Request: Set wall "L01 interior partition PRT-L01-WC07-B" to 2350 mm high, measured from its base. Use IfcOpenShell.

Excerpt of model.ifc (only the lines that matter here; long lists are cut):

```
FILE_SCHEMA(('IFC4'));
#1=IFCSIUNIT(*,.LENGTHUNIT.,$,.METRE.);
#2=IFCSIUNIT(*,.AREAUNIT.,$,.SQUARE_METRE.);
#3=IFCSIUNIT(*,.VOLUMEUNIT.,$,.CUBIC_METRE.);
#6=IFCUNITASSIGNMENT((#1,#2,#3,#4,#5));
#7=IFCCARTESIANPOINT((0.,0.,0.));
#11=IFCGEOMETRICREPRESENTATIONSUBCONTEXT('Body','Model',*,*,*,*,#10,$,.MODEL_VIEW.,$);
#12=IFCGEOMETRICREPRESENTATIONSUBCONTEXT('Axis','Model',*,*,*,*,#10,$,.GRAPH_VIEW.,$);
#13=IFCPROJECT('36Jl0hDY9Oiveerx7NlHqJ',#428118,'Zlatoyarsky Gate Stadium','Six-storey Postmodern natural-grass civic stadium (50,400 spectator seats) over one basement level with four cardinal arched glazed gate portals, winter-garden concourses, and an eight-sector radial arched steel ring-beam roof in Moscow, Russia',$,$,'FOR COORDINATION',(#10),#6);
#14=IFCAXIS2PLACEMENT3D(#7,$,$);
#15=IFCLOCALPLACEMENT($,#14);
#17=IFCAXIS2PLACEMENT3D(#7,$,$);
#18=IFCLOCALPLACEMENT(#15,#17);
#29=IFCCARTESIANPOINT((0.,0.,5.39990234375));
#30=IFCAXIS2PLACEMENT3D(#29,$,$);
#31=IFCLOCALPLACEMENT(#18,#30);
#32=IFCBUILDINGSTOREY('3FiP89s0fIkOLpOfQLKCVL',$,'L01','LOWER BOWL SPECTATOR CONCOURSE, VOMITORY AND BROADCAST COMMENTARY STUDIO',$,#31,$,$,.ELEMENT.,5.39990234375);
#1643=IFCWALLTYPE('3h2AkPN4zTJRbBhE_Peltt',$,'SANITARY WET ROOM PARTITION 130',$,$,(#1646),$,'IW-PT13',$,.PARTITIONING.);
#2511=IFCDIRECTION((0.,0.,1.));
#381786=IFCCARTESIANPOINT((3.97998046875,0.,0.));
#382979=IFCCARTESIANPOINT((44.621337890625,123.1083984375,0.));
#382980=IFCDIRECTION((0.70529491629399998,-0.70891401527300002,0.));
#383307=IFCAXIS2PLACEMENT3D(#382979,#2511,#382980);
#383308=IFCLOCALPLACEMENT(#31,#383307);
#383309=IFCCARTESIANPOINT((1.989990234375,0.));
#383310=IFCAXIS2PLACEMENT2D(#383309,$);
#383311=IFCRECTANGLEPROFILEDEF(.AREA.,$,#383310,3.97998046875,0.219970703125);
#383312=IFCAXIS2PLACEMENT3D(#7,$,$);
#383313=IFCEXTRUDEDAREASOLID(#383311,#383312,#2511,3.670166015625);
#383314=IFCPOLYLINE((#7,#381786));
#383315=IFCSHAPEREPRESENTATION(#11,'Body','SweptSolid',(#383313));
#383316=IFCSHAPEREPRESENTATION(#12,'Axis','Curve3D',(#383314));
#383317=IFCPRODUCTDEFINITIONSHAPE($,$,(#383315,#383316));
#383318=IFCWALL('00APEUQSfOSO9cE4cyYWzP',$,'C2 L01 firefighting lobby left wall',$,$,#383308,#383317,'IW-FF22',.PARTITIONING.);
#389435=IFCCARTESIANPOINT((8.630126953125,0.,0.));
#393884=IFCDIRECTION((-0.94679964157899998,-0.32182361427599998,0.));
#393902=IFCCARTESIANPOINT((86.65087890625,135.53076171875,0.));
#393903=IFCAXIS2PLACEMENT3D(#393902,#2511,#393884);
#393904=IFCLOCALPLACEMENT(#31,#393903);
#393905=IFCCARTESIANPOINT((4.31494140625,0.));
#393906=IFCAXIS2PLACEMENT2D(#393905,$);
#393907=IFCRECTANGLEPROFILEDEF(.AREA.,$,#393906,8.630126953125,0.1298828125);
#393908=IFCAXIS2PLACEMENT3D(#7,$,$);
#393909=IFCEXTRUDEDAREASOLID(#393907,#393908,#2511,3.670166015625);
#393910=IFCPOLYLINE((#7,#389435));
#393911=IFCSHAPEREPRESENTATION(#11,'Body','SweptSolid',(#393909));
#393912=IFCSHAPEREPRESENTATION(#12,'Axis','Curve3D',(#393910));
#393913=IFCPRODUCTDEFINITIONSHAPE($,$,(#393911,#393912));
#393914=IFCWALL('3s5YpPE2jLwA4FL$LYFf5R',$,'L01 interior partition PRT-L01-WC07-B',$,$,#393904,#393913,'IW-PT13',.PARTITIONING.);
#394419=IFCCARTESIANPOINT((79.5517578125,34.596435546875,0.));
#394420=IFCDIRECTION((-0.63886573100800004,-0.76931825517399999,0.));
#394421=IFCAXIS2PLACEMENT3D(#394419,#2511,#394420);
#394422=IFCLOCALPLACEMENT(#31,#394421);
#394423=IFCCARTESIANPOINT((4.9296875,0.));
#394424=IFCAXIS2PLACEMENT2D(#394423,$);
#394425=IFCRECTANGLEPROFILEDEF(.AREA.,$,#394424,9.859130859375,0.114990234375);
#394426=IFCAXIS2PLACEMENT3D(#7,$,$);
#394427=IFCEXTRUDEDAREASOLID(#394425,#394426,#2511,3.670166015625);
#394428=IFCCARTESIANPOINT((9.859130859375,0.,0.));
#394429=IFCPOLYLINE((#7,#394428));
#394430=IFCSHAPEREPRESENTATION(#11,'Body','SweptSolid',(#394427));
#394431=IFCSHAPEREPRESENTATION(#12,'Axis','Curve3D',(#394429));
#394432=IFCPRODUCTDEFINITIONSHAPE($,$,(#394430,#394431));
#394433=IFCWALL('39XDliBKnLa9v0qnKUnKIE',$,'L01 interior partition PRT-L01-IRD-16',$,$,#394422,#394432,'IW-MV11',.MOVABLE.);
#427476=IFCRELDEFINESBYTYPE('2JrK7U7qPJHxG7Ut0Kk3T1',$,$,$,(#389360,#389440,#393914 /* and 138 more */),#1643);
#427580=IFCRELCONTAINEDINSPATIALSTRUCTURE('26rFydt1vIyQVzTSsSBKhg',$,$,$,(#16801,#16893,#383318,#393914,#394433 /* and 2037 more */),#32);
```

```python
import ifcopenshell
import ifcopenshell.geom
import ifcopenshell.util.representation
import ifcopenshell.util.shape
import ifcopenshell.util.unit

model = ifcopenshell.open("model.ifc")
unit_scale = ifcopenshell.util.unit.calculate_unit_scale(model)
settings = ifcopenshell.geom.settings()


def volume(element):
    """Net volume in cubic metres, openings subtracted."""
    shape = ifcopenshell.geom.create_shape(settings, element)
    return ifcopenshell.util.shape.get_volume(shape.geometry)


wall = model.by_id(393914)
before = volume(wall)

body = ifcopenshell.util.representation.get_representation(wall, "Model", "Body")
solid = body.Items[0]
old_height = solid.Depth
solid.Depth = 2.35 / unit_scale
after = volume(wall)

print(f"height {old_height:g} -> {solid.Depth:g}, volume {before:.3f} -> {after:.3f} m3")

model.write("model_v2.ifc")
```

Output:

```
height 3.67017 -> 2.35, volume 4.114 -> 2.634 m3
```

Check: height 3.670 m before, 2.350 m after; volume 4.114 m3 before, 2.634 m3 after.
